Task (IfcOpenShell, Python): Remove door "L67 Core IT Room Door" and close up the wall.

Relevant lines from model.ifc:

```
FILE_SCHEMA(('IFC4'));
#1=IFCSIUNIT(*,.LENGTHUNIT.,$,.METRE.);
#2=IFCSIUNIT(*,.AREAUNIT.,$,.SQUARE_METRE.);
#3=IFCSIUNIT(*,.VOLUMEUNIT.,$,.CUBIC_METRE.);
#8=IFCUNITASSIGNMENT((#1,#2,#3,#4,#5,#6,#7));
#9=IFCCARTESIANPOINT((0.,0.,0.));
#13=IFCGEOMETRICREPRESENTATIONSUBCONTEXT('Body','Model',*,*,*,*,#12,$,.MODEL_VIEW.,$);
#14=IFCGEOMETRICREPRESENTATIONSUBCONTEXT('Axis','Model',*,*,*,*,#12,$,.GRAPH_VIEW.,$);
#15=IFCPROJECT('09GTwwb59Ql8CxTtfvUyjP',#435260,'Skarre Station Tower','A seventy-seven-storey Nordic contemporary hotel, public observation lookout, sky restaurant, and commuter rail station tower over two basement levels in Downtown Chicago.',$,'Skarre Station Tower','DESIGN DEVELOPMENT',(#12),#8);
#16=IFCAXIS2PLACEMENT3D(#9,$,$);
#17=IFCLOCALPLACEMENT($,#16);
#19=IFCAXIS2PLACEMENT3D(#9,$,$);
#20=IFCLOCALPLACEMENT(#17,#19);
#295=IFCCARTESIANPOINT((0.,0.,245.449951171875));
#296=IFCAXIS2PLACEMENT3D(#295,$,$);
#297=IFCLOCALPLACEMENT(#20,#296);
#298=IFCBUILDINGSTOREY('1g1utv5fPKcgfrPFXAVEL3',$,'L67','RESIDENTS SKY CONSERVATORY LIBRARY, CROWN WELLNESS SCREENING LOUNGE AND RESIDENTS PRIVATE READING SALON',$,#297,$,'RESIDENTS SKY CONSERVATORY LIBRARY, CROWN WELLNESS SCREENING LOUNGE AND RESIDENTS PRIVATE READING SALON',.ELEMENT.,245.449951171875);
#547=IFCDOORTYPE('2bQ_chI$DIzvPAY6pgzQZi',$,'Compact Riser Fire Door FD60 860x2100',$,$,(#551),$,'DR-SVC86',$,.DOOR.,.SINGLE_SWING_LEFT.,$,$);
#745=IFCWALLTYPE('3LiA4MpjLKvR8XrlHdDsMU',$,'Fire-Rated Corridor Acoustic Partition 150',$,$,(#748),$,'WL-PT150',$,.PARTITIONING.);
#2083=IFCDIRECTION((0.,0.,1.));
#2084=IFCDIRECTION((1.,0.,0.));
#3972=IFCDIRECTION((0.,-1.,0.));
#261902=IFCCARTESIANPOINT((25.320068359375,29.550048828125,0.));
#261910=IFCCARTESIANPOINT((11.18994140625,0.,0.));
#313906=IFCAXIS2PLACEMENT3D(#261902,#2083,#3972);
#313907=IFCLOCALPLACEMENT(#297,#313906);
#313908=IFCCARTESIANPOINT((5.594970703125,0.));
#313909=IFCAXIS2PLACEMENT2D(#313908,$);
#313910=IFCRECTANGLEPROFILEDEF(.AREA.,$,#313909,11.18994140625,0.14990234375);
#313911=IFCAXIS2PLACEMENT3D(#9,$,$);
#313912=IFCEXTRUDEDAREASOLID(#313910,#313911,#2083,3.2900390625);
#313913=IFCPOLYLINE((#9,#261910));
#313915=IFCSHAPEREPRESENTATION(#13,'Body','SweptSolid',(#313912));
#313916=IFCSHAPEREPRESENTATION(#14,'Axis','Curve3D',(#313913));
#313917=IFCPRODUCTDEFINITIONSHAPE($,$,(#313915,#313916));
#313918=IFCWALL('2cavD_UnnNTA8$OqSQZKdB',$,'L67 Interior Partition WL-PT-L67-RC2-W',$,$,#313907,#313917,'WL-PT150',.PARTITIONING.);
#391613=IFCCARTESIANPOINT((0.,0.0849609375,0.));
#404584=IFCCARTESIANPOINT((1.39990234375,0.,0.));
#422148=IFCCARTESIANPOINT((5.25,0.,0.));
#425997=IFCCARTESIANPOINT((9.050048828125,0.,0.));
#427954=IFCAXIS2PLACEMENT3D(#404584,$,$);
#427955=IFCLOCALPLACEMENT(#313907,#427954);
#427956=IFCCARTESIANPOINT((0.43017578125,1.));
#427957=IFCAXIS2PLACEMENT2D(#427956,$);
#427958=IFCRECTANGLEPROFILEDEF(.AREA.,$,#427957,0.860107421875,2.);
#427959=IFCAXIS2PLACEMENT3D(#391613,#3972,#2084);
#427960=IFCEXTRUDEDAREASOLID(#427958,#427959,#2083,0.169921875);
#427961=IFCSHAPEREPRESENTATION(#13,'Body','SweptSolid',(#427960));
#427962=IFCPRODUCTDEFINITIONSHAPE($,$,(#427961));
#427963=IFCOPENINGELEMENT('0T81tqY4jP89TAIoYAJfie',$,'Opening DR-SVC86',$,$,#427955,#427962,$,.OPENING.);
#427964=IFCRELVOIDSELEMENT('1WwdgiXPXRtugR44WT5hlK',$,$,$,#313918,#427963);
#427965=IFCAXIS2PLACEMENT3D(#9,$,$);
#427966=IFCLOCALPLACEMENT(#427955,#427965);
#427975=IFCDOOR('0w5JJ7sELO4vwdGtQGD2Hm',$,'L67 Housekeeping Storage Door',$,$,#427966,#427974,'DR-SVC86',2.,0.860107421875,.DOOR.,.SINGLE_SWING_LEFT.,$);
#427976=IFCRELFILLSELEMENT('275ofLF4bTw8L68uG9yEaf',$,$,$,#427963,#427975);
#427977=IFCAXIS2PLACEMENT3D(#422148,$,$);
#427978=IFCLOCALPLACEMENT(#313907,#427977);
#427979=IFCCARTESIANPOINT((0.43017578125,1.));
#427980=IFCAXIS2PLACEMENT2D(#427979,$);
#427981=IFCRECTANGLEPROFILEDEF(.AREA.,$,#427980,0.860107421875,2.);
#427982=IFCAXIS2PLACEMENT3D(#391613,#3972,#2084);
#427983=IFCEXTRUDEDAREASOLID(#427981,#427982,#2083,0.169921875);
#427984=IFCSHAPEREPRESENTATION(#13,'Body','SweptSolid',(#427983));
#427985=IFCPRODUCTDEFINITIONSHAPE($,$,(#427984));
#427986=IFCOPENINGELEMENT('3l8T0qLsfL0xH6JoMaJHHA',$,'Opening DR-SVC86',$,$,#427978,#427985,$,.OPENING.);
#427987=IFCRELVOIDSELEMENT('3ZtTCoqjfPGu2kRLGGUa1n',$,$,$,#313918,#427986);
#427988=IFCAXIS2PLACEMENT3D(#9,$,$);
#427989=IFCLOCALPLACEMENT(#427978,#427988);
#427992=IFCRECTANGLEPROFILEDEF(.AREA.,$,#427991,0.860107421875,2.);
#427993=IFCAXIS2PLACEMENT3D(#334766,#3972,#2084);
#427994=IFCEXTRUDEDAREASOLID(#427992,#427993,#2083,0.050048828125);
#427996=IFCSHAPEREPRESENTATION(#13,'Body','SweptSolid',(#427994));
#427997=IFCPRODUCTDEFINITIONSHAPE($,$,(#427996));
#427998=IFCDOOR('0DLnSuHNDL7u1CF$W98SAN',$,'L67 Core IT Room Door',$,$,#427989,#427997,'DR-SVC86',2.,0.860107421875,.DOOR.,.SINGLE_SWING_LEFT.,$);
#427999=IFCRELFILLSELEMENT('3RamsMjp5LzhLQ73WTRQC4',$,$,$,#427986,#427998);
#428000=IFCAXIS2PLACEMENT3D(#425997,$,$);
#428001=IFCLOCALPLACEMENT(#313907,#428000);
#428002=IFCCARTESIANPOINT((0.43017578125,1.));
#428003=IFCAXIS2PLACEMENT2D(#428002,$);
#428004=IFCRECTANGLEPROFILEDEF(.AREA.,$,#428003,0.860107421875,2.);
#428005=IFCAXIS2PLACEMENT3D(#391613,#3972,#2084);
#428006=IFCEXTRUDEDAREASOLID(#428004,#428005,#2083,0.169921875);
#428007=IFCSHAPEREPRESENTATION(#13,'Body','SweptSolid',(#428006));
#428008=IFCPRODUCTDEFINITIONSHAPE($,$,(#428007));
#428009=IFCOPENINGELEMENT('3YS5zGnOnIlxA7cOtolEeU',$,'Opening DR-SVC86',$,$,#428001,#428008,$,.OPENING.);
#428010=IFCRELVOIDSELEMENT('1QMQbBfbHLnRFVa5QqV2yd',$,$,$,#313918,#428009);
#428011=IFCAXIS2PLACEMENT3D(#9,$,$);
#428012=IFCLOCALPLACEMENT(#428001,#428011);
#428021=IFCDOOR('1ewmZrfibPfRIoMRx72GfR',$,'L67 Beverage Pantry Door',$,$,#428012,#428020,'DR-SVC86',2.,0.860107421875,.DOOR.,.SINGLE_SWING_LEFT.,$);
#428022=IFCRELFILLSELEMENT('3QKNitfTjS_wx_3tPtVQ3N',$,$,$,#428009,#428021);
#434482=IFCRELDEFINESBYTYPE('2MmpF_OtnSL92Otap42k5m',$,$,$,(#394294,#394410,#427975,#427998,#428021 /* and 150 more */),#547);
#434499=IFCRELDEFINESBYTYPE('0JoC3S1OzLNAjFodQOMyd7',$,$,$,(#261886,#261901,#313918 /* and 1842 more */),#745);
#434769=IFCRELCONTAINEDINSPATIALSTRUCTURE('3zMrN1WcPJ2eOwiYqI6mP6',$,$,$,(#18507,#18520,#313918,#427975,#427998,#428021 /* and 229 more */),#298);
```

```python
import ifcopenshell
import ifcopenshell.api.feature
import ifcopenshell.api.root
import ifcopenshell.geom
import ifcopenshell.util.shape

model = ifcopenshell.open("model.ifc")
settings = ifcopenshell.geom.settings()


def volume(element):
    """Net volume in cubic metres, openings subtracted."""
    shape = ifcopenshell.geom.create_shape(settings, element)
    return ifcopenshell.util.shape.get_volume(shape.geometry)


door = model.by_guid("0DLnSuHNDL7u1CF$W98SAN")
opening = door.FillsVoids[0].RelatingOpeningElement
wall = opening.VoidsElements[0].RelatingBuildingElement
before = volume(wall)

ifcopenshell.api.root.remove_product(model, product=door)
ifcopenshell.api.feature.remove_feature(model, feature=opening)

after = volume(wall)

print(f"wall volume {before:.3f} -> {after:.3f} m3")

model.write("model_updated.ifc")
```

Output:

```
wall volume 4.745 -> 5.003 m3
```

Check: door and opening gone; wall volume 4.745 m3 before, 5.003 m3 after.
